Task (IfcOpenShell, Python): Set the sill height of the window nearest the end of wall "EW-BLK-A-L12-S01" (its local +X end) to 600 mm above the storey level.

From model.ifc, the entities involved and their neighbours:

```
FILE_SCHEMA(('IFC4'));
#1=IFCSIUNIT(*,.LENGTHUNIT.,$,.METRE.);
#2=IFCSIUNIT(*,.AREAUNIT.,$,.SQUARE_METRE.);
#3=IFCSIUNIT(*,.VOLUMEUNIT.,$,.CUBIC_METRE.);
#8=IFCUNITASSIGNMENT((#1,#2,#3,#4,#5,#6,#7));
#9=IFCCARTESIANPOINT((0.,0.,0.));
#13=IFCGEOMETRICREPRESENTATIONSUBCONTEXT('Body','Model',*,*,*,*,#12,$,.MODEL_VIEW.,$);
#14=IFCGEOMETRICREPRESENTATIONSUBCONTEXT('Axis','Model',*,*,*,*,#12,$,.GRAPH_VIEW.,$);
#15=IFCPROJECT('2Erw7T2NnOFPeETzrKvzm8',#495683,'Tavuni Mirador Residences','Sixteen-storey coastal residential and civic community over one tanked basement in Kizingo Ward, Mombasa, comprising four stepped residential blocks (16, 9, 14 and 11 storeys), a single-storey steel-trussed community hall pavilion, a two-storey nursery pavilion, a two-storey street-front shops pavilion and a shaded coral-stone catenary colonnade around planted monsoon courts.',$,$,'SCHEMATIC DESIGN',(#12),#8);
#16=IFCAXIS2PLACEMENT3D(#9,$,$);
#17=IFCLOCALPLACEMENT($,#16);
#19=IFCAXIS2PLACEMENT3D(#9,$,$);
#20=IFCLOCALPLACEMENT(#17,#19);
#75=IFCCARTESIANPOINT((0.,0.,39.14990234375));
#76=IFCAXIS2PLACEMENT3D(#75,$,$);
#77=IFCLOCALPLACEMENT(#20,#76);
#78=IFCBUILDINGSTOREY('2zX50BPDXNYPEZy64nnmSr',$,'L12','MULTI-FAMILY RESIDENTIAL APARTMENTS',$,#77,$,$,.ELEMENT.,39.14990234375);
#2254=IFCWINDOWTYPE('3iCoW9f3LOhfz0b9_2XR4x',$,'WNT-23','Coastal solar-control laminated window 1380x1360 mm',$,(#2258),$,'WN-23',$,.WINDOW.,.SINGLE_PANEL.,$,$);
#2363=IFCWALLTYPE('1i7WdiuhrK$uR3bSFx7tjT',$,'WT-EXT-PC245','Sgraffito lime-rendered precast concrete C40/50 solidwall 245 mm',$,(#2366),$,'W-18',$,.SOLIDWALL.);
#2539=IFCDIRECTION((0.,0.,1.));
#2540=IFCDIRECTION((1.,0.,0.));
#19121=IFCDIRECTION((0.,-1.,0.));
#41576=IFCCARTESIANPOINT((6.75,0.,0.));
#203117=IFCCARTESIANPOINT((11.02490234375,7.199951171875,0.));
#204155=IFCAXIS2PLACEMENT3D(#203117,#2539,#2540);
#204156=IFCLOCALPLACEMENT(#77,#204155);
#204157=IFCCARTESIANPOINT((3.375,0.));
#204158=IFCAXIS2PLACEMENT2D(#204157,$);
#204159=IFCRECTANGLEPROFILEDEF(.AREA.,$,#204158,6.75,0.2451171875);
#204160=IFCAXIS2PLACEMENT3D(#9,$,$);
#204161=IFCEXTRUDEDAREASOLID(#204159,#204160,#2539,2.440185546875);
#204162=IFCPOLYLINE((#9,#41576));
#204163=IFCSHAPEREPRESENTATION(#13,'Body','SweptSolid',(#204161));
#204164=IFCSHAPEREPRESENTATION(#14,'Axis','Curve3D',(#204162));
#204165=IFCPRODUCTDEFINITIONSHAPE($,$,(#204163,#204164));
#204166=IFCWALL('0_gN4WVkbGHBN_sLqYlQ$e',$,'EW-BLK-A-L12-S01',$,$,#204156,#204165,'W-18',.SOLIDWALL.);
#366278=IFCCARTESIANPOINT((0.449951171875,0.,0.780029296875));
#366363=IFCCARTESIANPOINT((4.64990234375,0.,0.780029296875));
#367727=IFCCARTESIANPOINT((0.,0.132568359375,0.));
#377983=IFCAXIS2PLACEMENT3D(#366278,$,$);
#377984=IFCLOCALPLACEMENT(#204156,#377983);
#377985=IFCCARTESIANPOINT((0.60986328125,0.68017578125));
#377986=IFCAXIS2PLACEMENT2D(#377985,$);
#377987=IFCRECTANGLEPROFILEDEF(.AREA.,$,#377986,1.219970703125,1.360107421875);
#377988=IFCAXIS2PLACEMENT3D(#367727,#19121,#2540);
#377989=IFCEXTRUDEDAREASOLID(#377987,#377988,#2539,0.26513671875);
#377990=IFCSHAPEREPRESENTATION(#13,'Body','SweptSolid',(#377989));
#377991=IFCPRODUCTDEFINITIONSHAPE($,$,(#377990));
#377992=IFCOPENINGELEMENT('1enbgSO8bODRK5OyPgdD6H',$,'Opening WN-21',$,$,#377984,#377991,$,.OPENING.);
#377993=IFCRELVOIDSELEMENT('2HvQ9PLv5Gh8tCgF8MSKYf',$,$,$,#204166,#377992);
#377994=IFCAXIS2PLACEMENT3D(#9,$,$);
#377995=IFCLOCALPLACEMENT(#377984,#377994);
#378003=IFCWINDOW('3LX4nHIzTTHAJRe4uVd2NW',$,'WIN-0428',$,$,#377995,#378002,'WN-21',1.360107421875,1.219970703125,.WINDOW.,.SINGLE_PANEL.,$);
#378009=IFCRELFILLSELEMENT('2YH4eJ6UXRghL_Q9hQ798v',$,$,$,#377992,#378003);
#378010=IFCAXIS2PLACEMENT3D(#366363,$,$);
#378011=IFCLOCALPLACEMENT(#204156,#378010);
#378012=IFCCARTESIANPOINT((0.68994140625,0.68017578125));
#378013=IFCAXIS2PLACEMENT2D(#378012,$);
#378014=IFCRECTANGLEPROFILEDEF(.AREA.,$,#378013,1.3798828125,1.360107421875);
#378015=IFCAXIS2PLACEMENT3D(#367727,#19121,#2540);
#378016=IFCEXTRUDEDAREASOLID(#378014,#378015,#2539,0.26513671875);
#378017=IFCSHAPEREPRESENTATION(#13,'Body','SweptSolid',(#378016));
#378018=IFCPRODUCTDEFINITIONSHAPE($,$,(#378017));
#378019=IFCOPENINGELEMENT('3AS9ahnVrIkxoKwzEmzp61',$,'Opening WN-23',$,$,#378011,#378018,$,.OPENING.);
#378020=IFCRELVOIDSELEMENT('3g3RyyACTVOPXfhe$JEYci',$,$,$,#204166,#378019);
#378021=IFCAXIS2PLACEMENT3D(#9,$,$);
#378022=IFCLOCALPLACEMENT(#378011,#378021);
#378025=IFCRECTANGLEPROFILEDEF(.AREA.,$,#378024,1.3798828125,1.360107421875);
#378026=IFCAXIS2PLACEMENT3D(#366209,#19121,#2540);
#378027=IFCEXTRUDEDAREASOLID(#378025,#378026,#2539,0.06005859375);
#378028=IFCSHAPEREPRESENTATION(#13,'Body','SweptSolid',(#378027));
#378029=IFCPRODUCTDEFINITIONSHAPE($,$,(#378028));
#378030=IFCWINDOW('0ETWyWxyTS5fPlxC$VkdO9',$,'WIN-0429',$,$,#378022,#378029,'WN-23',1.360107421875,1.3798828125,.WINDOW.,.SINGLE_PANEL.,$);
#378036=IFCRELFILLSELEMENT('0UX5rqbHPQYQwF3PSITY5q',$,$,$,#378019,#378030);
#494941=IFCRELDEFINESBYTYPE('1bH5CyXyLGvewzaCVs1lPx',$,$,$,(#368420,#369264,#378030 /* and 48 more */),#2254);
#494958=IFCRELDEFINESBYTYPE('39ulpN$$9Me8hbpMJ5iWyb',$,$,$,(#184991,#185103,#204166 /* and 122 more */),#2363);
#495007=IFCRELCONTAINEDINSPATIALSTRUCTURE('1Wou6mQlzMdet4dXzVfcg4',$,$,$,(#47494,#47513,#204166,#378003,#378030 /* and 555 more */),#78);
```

```python
import numpy as np
import ifcopenshell
import ifcopenshell.api.geometry
import ifcopenshell.geom
import ifcopenshell.util.element
import ifcopenshell.util.placement
import ifcopenshell.util.shape
import ifcopenshell.util.unit

model = ifcopenshell.open("model.ifc")
unit_scale = ifcopenshell.util.unit.calculate_unit_scale(model)

window = model.by_guid("0ETWyWxyTS5fPlxC$VkdO9")
opening = window.FillsVoids[0].RelatingOpeningElement
storey = ifcopenshell.util.element.get_container(window, ifc_class="IfcBuildingStorey")
level = ifcopenshell.util.placement.get_local_placement(storey.ObjectPlacement)[2, 3]

# The opening's origin need not be at the sill, so measure its lowest point.
shape = ifcopenshell.geom.create_shape(ifcopenshell.geom.settings(), opening)
bottom = ifcopenshell.util.shape.get_shape_bottom_elevation(shape, shape.geometry) / unit_scale
dz = level + 0.6 / unit_scale - bottom

shift = np.array([0.0, 0.0, dz])
# The window is placed relative to its opening, so it follows when the opening moves.
matrix = ifcopenshell.util.placement.get_local_placement(opening.ObjectPlacement)
matrix[:3, 3] += shift
ifcopenshell.api.geometry.edit_object_placement(
    model, product=opening, matrix=matrix, is_si=False, should_transform_children=True
)

print(f"moved by {dz * unit_scale:+.3f} m")

model.write("model_v2.ifc")
```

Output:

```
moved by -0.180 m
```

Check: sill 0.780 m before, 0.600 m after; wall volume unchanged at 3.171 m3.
